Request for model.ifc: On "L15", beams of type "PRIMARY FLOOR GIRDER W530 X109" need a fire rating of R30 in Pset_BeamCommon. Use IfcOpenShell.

First a look at what the model holds.

```python
import ifcopenshell
import ifcopenshell.util.element

model = ifcopenshell.open("model.ifc")
print(model.schema)
storey = next(s for s in model.by_type("IfcBuildingStorey") if s.Name == "L15")
beams = [e for e in ifcopenshell.util.element.get_decomposition(storey) if e.is_a("IfcBeam")]
seen = {}
for e in beams:
    element_type = ifcopenshell.util.element.get_type(e)
    key = (element_type.Name if element_type != e and element_type else None, ifcopenshell.util.element.get_pset(e, "Pset_BeamCommon", "FireRating"))
    seen[key] = seen.get(key, 0) + 1
for (name, value), count in sorted(seen.items(), key=str):
    print(count, "x", name, "|", value)
```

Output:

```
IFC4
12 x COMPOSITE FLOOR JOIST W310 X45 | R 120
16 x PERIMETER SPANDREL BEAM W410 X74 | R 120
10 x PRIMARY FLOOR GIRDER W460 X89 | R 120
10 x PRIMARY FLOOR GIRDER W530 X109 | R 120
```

```python
import ifcopenshell
import ifcopenshell.api.pset
import ifcopenshell.util.element

model = ifcopenshell.open("model.ifc")

storey = next(s for s in model.by_type("IfcBuildingStorey") if s.Name == "L15")
beams = [e for e in ifcopenshell.util.element.get_decomposition(storey) if e.is_a("IfcBeam")]

count = 0
for e in beams:
    element_type = ifcopenshell.util.element.get_type(e)
    if element_type in (None, e) or element_type.Name != "PRIMARY FLOOR GIRDER W530 X109":
        continue
    # add_pset returns the element's existing set when there is one.
    pset = ifcopenshell.api.pset.add_pset(model, product=e, name="Pset_BeamCommon")
    ifcopenshell.api.pset.edit_pset(model, pset=pset, properties={"FireRating": "R30"})
    count += 1

print(count, "beams updated")

model.write("model-out.ifc")
```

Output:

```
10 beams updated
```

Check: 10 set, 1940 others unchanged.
